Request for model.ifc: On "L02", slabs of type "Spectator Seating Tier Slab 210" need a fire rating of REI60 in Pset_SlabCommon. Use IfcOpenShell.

First a look at what the model holds.

```python
import ifcopenshell
import ifcopenshell.util.element

model = ifcopenshell.open("model.ifc")
print(model.schema)
storey = next(s for s in model.by_type("IfcBuildingStorey") if s.Name == "L02")
slabs = [e for e in ifcopenshell.util.element.get_decomposition(storey) if e.is_a("IfcSlab")]
seen = {}
for e in slabs:
    element_type = ifcopenshell.util.element.get_type(e)
    key = (element_type.Name if element_type != e and element_type else None, ifcopenshell.util.element.get_pset(e, "Pset_SlabCommon", "FireRating"))
    seen[key] = seen.get(key, 0) + 1
for (name, value), count in sorted(seen.items(), key=str):
    print(count, "x", name, "|", value)
```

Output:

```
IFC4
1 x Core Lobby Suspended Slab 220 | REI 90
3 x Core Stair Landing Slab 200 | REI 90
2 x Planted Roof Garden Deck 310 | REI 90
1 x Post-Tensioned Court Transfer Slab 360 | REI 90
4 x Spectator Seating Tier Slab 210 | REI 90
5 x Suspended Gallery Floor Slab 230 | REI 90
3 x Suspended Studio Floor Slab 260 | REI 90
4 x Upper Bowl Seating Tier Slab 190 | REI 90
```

```python
import ifcopenshell
import ifcopenshell.api.pset
import ifcopenshell.util.element

model = ifcopenshell.open("model.ifc")

storey = next(s for s in model.by_type("IfcBuildingStorey") if s.Name == "L02")
slabs = [e for e in ifcopenshell.util.element.get_decomposition(storey) if e.is_a("IfcSlab")]

count = 0
for e in slabs:
    element_type = ifcopenshell.util.element.get_type(e)
    if element_type in (None, e) or element_type.Name != "Spectator Seating Tier Slab 210":
        continue
    # add_pset returns the element's existing set when there is one.
    pset = ifcopenshell.api.pset.add_pset(model, product=e, name="Pset_SlabCommon")
    ifcopenshell.api.pset.edit_pset(model, pset=pset, properties={"FireRating": "REI60"})
    count += 1

print(count, "slabs updated")

model.write("model_v2.ifc")
```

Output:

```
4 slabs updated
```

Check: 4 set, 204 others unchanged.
